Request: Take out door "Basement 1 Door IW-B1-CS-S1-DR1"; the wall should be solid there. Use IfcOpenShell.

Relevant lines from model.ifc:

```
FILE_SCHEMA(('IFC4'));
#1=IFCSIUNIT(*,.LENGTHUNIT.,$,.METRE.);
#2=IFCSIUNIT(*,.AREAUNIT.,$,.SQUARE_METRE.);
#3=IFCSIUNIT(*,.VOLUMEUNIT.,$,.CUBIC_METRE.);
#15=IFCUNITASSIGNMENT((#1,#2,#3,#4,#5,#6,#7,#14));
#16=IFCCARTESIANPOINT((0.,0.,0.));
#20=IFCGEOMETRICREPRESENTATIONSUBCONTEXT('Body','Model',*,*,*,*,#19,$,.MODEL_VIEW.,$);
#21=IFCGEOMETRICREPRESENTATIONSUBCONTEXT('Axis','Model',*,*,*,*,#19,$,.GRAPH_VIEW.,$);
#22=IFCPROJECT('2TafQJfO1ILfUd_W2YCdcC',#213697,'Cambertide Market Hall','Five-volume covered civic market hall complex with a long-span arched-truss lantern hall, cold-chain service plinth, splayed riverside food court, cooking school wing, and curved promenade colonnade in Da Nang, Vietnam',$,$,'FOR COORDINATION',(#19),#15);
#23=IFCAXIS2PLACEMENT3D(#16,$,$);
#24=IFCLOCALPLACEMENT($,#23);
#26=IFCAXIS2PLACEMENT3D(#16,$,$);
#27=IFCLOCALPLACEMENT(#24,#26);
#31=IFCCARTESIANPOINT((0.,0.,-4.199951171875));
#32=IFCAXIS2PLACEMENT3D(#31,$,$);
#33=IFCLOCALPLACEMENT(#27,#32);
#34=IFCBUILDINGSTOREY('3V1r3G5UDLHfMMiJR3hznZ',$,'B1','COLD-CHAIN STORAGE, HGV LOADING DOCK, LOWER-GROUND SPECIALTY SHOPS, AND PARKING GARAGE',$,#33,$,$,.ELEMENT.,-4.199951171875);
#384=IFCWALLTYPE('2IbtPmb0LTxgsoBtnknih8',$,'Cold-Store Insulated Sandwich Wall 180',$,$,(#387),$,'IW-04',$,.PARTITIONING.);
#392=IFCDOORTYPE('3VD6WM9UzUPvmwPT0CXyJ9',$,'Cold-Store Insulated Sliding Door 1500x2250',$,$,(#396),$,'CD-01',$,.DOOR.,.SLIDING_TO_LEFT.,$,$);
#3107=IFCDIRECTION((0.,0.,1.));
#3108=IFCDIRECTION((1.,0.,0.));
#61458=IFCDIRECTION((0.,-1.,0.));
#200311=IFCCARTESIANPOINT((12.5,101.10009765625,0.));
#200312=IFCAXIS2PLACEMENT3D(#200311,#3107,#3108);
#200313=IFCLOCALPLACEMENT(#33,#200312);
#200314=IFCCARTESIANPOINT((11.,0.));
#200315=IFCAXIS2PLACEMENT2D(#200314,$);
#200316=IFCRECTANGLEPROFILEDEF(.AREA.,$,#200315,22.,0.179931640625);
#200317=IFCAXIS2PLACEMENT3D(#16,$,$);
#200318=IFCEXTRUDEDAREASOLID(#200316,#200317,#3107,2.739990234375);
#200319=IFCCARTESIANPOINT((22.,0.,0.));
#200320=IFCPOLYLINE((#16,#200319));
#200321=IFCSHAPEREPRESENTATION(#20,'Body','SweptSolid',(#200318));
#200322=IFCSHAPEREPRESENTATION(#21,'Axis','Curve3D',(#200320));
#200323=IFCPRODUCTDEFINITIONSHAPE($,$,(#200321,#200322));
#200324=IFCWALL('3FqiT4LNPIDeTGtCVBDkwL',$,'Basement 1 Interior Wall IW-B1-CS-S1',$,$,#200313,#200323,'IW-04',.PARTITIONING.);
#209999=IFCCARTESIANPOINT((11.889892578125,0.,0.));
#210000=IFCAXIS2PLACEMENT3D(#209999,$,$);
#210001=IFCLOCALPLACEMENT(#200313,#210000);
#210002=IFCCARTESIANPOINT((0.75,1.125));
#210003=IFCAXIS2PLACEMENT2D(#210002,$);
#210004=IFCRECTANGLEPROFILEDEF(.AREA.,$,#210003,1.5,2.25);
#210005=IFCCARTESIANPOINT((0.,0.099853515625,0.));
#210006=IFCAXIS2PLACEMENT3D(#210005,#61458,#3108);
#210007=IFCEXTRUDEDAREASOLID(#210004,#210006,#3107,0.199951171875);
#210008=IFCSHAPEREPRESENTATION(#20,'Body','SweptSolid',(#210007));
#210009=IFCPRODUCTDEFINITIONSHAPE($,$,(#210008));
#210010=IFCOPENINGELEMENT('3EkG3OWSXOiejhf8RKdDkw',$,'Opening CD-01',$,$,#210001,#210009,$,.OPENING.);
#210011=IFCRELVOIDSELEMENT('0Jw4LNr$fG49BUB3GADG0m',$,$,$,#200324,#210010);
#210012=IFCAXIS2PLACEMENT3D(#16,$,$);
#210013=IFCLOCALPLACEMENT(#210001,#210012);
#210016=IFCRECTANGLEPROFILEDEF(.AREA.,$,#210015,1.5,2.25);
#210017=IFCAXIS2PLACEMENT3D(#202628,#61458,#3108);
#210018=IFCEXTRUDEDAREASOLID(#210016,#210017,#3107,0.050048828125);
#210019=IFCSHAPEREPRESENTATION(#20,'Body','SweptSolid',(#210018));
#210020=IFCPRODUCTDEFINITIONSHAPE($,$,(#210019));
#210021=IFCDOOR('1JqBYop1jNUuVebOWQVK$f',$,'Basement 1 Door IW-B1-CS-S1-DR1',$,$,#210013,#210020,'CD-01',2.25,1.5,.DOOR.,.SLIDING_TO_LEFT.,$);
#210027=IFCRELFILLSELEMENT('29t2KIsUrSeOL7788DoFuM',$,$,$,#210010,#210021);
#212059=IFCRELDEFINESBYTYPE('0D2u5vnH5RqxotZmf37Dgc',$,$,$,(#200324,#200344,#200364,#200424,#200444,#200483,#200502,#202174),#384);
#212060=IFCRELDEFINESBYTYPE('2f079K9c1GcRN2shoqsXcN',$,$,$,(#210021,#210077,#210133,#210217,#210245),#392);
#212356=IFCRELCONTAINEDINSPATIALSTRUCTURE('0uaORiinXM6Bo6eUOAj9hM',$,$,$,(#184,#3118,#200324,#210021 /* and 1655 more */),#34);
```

```python
import ifcopenshell
import ifcopenshell.api.feature
import ifcopenshell.api.root
import ifcopenshell.geom
import ifcopenshell.util.shape

model = ifcopenshell.open("model.ifc")
settings = ifcopenshell.geom.settings()


def volume(element):
    """Net volume in cubic metres, openings subtracted."""
    shape = ifcopenshell.geom.create_shape(settings, element)
    return ifcopenshell.util.shape.get_volume(shape.geometry)


door = model.by_id(210021)
opening = door.FillsVoids[0].RelatingOpeningElement
wall = opening.VoidsElements[0].RelatingBuildingElement
before = volume(wall)

ifcopenshell.api.root.remove_product(model, product=door)
ifcopenshell.api.feature.remove_feature(model, feature=opening)

after = volume(wall)

print(f"wall volume {before:.3f} -> {after:.3f} m3")

model.write("model-out.ifc")
```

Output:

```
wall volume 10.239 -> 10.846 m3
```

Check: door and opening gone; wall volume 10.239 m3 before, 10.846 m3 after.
